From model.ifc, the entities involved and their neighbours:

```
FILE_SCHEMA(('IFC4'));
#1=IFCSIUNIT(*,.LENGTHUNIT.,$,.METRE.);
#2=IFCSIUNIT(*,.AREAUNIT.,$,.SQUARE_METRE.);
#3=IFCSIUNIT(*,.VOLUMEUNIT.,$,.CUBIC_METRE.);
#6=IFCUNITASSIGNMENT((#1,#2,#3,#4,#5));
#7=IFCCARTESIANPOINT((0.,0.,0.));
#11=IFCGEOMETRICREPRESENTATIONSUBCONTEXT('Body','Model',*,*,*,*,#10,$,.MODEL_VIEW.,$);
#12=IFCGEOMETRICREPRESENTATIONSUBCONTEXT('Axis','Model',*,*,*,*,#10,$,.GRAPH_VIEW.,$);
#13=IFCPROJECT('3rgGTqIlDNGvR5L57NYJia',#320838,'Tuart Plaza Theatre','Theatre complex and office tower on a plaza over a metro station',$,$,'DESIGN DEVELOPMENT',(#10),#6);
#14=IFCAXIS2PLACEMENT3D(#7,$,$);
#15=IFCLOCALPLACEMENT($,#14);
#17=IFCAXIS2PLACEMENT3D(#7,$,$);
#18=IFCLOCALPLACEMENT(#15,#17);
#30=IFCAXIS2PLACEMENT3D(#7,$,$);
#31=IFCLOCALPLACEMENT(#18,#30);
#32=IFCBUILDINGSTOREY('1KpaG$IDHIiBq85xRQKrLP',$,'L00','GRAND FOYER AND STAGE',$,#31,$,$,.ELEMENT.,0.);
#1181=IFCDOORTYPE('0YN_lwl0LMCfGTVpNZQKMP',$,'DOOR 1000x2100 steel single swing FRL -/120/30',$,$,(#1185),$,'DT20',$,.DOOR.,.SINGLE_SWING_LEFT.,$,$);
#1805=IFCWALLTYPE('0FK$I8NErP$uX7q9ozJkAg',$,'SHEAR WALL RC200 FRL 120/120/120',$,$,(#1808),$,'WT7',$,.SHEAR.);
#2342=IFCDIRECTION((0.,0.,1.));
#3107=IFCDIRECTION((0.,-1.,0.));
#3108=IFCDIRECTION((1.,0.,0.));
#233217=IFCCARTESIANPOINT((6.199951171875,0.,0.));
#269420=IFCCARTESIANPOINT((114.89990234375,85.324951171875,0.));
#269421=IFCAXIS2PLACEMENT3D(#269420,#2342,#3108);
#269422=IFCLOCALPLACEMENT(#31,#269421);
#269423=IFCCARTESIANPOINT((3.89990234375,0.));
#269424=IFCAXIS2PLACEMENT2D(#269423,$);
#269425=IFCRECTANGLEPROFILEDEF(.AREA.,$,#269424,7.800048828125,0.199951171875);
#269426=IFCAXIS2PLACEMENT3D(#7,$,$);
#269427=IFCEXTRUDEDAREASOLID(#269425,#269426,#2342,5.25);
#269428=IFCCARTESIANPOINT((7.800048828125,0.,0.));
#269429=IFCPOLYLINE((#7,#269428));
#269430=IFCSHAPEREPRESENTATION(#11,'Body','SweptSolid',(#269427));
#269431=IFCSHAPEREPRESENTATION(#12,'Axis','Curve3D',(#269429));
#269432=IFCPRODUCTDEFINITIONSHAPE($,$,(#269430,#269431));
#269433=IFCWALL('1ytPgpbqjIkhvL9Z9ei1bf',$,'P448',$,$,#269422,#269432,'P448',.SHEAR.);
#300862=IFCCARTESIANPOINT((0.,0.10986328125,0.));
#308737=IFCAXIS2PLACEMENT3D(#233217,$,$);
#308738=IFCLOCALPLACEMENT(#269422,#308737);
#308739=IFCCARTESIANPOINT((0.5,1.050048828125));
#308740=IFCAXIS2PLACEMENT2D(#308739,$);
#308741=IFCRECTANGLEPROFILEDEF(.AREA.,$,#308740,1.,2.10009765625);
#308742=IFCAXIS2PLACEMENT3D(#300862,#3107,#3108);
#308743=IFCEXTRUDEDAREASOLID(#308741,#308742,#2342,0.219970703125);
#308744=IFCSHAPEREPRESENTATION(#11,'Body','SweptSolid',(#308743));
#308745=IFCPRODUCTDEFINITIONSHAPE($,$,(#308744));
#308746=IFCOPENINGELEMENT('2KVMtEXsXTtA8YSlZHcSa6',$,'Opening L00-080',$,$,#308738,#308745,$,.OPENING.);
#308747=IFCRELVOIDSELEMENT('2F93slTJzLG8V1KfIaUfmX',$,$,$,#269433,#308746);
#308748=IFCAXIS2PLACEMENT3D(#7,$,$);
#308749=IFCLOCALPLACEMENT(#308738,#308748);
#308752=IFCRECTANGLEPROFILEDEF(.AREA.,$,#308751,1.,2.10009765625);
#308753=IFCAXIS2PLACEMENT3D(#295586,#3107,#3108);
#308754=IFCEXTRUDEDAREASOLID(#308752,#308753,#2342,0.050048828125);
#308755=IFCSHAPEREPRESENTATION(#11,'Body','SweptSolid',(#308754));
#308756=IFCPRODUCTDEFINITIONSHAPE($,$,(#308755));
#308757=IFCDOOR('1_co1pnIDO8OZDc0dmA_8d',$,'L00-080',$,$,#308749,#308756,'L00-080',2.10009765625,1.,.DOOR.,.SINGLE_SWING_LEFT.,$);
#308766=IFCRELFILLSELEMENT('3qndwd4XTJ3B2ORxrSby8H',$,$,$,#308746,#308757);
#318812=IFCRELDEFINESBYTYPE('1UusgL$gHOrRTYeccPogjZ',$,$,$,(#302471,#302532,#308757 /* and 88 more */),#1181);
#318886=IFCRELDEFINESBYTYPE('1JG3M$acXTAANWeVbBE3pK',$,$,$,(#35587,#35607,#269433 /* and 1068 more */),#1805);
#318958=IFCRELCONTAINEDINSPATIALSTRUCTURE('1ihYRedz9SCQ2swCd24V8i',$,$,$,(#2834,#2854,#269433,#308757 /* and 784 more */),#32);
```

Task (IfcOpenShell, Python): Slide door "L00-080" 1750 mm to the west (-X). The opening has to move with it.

```python
import ifcopenshell
import ifcopenshell.api.geometry
import ifcopenshell.util.placement

model = ifcopenshell.open("model.ifc")

door = model.by_guid("1_co1pnIDO8OZDc0dmA_8d")
opening = door.FillsVoids[0].RelatingOpeningElement
wall = opening.VoidsElements[0].RelatingBuildingElement

wall_matrix = ifcopenshell.util.placement.get_local_placement(wall.ObjectPlacement)
shift = wall_matrix[:3, 0] * -1.75
before = ifcopenshell.util.placement.get_local_placement(door.ObjectPlacement)[:3, 3].copy()

# The door is placed relative to its opening, so it follows when the opening moves.
matrix = ifcopenshell.util.placement.get_local_placement(opening.ObjectPlacement)
matrix[:3, 3] += shift
ifcopenshell.api.geometry.edit_object_placement(
    model, product=opening, matrix=matrix, is_si=False, should_transform_children=True
)

after = ifcopenshell.util.placement.get_local_placement(door.ObjectPlacement)[:3, 3]
print("door moved by", (after - before).round(3) + 0.0)

model.write("model_rev.ifc")
```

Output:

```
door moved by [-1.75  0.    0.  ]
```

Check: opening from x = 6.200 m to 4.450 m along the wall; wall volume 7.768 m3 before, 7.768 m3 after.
